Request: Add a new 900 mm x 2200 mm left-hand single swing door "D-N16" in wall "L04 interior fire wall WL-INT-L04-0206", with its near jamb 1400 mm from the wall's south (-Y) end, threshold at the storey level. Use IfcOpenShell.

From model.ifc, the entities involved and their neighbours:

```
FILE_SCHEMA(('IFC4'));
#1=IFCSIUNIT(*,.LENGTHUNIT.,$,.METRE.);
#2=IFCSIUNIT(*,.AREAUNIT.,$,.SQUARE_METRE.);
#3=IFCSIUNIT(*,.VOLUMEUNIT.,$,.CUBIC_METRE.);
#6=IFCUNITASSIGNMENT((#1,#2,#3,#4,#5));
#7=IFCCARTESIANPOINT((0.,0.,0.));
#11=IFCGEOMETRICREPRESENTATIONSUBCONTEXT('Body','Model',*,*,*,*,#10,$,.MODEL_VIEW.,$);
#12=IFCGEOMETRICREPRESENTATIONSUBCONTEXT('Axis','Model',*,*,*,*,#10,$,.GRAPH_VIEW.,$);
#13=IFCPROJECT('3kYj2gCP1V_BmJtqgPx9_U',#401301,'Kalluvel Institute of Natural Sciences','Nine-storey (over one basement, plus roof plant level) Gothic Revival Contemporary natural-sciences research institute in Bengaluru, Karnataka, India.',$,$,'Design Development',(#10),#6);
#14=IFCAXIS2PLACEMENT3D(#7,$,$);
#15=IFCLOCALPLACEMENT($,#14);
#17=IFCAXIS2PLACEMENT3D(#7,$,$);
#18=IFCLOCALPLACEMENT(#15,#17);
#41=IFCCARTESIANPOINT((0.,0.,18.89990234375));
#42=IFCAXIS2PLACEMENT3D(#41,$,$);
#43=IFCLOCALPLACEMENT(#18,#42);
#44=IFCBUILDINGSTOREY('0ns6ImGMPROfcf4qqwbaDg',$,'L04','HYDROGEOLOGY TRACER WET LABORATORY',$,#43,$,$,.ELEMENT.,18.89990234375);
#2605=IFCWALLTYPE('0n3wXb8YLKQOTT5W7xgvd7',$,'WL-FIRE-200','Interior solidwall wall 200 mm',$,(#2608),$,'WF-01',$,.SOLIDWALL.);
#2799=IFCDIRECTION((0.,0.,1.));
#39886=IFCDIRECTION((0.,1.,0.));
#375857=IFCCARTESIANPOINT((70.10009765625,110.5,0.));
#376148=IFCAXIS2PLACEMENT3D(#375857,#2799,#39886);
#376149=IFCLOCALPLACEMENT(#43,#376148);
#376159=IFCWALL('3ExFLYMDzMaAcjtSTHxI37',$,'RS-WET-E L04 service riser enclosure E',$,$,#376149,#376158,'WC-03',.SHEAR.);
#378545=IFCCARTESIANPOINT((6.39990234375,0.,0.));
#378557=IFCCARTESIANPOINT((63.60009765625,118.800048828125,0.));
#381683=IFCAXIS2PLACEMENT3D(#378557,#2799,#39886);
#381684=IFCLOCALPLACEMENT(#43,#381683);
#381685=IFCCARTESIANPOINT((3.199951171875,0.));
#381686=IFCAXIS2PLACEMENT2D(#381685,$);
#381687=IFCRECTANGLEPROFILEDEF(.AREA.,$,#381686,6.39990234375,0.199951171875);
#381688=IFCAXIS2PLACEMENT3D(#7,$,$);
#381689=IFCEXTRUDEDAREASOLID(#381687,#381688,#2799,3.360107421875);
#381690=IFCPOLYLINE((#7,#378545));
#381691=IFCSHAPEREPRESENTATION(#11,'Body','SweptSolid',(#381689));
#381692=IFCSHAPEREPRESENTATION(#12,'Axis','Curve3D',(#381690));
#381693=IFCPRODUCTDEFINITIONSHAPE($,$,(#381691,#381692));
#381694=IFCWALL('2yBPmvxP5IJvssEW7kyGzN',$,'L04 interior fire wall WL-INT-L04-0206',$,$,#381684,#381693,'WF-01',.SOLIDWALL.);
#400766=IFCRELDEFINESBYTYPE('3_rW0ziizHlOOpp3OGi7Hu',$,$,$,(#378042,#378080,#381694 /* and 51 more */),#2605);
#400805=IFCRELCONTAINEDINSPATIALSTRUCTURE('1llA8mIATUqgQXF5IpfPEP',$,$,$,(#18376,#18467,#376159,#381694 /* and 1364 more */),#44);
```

```python
import numpy as np
import ifcopenshell
import ifcopenshell.api.feature
import ifcopenshell.api.geometry
import ifcopenshell.api.root
import ifcopenshell.api.spatial
import ifcopenshell.geom
import ifcopenshell.util.element
import ifcopenshell.util.placement
import ifcopenshell.util.representation
import ifcopenshell.util.shape
import ifcopenshell.util.unit

model = ifcopenshell.open("model.ifc")
unit_scale = ifcopenshell.util.unit.calculate_unit_scale(model)
settings = ifcopenshell.geom.settings()


def volume(element):
    """Net volume in cubic metres, openings subtracted."""
    shape = ifcopenshell.geom.create_shape(settings, element)
    return ifcopenshell.util.shape.get_volume(shape.geometry)


wall = model.by_guid("2yBPmvxP5IJvssEW7kyGzN")
storey = ifcopenshell.util.element.get_container(wall, ifc_class="IfcBuildingStorey")
context = ifcopenshell.util.representation.get_context(model, "Model", "Body", "MODEL_VIEW")
before = volume(wall)

width, height, from_end, sill = 0.9, 2.2, 1.4, 0.0  # metres

# The wall runs along its own X axis, and the end named is its -X end.
wall_shape = ifcopenshell.geom.create_shape(settings, wall)
x, y, z = ifcopenshell.util.shape.get_vertices(wall_shape.geometry).T
start = x.min() + from_end
face, thickness = float(y.min()), float(y.max() - y.min())
wall_matrix = ifcopenshell.util.placement.get_local_placement(wall.ObjectPlacement)
level = ifcopenshell.util.placement.get_local_placement(storey.ObjectPlacement)[2, 3]


def in_wall(x, y):
    """Placement at x, y metres in the wall's axes, at sill height."""
    matrix = wall_matrix.copy()
    matrix[:, 3] = wall_matrix @ np.array([x / unit_scale, y / unit_scale, 0.0, 1.0])
    matrix[2, 3] = level + sill / unit_scale
    return matrix


# Opening: a box that overshoots both wall faces by 50 mm.
opening = ifcopenshell.api.root.create_entity(model, ifc_class="IfcOpeningElement", predefined_type="OPENING")
box = ifcopenshell.api.geometry.add_wall_representation(
    model, context=context, length=width, height=height, thickness=thickness + 0.1
)
ifcopenshell.api.geometry.assign_representation(model, product=opening, representation=box)
ifcopenshell.api.geometry.edit_object_placement(model, product=opening, matrix=in_wall(start, face - 0.05), is_si=False)
ifcopenshell.api.feature.add_feature(model, feature=opening, element=wall)

door = ifcopenshell.api.root.create_entity(model, ifc_class="IfcDoor", name="D-N16", predefined_type="DOOR")
door.OverallWidth, door.OverallHeight = width / unit_scale, height / unit_scale
door.OperationType = "SINGLE_SWING_LEFT"
body = ifcopenshell.api.geometry.add_door_representation(
    model,
    context=context,
    overall_width=door.OverallWidth,
    overall_height=door.OverallHeight,
    operation_type="SINGLE_SWING_LEFT",
    lining_properties={"LiningDepth": thickness / unit_scale, "ThresholdDepth": thickness / unit_scale},
)
ifcopenshell.api.geometry.assign_representation(model, product=door, representation=body)
ifcopenshell.api.spatial.assign_container(model, products=[door], relating_structure=storey)
ifcopenshell.api.feature.add_filling(model, opening=opening, element=door)

# The lining spans the wall, so the door starts at the wall face.
ifcopenshell.api.geometry.edit_object_placement(model, product=door, matrix=in_wall(start, face), is_si=False)

after = volume(wall)

print(f"wall volume {before:.3f} -> {after:.3f} m3")

model.write("model_v2.ifc")
```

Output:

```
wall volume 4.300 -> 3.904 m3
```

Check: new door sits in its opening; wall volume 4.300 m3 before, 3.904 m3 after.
